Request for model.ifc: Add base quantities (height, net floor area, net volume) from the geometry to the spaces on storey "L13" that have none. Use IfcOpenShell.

First a look at what the model holds.

```python
import ifcopenshell
import ifcopenshell.util.element
import ifcopenshell.util.unit

model = ifcopenshell.open("model.ifc")
print(model.schema)
for unit_type in ("LENGTHUNIT", "AREAUNIT", "VOLUMEUNIT"):
    print(unit_type, ifcopenshell.util.unit.calculate_unit_scale(model, unit_type))
storey = next(s for s in model.by_type("IfcBuildingStorey") if s.Name == "L13")
spaces = [e for e in ifcopenshell.util.element.get_decomposition(storey) if e.is_a("IfcSpace")]
for e in sorted(spaces, key=lambda e: e.id()):
    print(e.id(), e.is_a(), e.Name, list(ifcopenshell.util.element.get_psets(e, qtos_only=True)), sep=" | ")
```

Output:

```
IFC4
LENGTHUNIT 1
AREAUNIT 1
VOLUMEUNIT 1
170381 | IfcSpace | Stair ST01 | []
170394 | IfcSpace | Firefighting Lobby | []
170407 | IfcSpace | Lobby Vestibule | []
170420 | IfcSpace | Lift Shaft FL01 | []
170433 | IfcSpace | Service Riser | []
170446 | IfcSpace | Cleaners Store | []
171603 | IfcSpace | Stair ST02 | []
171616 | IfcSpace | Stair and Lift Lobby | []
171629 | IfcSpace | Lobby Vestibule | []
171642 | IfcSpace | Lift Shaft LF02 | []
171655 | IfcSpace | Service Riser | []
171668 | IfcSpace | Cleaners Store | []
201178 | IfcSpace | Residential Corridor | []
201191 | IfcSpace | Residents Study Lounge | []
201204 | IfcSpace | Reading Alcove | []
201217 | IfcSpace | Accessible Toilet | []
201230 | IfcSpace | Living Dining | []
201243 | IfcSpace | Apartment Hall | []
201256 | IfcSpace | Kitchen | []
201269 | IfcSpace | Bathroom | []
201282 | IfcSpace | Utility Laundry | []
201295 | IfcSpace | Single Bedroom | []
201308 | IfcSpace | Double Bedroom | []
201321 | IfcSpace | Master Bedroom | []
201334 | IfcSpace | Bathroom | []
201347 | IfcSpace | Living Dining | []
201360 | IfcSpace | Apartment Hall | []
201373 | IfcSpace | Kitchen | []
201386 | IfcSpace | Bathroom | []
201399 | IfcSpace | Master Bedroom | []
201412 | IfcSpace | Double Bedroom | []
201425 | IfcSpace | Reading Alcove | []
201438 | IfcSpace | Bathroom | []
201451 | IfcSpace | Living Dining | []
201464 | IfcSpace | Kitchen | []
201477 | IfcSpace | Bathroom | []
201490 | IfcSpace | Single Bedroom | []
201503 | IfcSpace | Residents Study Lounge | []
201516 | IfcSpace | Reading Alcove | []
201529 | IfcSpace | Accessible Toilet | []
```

```python
import ifcopenshell
import ifcopenshell.api.pset
import ifcopenshell.geom
import ifcopenshell.util.element
import ifcopenshell.util.shape
import ifcopenshell.util.unit

model = ifcopenshell.open("model.ifc")
unit_scale = ifcopenshell.util.unit.calculate_unit_scale(model)
area_scale = ifcopenshell.util.unit.calculate_unit_scale(model, "AREAUNIT")
volume_scale = ifcopenshell.util.unit.calculate_unit_scale(model, "VOLUMEUNIT")
settings = ifcopenshell.geom.settings()

storey = next(s for s in model.by_type("IfcBuildingStorey") if s.Name == "L13")
spaces = [e for e in ifcopenshell.util.element.get_decomposition(storey) if e.is_a("IfcSpace")]

for e in sorted(spaces, key=lambda e: e.id()):
    if ifcopenshell.util.element.get_psets(e, qtos_only=True, should_inherit=False):
        continue
    # Geometry comes back in metres, in the element's own axes.
    shape = ifcopenshell.geom.create_shape(settings, e)
    values = {
        "Height": ifcopenshell.util.shape.get_z(shape.geometry) / unit_scale,
        "NetFloorArea": ifcopenshell.util.shape.get_footprint_area(shape.geometry) / area_scale,
        "NetVolume": ifcopenshell.util.shape.get_volume(shape.geometry) / volume_scale,
    }
    qto = ifcopenshell.api.pset.add_qto(model, product=e, name="Qto_SpaceBaseQuantities")
    ifcopenshell.api.pset.edit_qto(model, qto=qto, properties=values)
    print(e.id(), {k: round(v, 3) for k, v in values.items()})

model.write("model_updated.ifc")
```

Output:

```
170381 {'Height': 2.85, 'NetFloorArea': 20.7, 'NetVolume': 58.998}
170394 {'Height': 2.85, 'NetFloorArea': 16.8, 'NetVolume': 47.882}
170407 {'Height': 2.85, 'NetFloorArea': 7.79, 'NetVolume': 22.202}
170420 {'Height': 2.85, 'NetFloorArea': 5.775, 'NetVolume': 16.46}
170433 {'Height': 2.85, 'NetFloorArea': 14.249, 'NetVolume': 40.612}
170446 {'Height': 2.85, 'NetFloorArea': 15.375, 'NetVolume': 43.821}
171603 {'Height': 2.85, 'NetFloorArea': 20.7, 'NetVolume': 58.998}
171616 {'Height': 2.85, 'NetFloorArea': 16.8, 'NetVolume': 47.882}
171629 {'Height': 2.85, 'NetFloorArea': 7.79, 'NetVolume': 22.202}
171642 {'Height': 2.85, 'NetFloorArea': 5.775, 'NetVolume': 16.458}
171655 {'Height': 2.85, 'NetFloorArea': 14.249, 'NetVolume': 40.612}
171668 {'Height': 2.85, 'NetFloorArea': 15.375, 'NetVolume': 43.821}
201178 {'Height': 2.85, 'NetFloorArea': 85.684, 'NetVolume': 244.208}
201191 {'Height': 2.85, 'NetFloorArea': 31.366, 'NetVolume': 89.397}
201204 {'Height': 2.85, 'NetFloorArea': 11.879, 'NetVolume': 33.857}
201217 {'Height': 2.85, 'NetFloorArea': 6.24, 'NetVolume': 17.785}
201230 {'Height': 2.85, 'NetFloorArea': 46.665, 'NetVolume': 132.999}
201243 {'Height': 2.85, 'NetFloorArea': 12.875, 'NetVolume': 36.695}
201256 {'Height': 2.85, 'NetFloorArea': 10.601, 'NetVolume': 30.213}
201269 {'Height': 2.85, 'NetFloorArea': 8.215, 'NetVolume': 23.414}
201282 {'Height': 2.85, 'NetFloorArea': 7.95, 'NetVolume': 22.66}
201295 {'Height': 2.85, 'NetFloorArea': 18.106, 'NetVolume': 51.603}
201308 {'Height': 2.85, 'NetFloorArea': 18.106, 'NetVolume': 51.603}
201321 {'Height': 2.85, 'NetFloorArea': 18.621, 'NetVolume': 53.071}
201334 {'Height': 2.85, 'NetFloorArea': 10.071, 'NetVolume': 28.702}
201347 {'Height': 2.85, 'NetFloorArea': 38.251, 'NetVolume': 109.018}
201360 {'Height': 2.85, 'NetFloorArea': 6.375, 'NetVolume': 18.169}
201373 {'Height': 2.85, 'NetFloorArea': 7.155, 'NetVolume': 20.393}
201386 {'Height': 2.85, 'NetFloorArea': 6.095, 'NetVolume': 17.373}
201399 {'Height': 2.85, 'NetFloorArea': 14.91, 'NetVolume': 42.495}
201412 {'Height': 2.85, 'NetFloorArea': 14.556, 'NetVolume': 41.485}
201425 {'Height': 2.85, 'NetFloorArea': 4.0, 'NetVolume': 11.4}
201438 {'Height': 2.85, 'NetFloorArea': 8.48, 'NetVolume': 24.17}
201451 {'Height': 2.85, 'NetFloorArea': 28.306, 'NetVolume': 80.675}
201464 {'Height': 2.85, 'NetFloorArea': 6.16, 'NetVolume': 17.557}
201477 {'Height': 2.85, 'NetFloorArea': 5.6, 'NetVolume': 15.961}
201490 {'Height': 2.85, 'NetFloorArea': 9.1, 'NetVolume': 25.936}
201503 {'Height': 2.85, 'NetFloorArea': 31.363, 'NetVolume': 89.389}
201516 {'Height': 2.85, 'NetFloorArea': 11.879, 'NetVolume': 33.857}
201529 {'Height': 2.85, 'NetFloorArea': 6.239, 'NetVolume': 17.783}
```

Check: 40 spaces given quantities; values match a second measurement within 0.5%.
